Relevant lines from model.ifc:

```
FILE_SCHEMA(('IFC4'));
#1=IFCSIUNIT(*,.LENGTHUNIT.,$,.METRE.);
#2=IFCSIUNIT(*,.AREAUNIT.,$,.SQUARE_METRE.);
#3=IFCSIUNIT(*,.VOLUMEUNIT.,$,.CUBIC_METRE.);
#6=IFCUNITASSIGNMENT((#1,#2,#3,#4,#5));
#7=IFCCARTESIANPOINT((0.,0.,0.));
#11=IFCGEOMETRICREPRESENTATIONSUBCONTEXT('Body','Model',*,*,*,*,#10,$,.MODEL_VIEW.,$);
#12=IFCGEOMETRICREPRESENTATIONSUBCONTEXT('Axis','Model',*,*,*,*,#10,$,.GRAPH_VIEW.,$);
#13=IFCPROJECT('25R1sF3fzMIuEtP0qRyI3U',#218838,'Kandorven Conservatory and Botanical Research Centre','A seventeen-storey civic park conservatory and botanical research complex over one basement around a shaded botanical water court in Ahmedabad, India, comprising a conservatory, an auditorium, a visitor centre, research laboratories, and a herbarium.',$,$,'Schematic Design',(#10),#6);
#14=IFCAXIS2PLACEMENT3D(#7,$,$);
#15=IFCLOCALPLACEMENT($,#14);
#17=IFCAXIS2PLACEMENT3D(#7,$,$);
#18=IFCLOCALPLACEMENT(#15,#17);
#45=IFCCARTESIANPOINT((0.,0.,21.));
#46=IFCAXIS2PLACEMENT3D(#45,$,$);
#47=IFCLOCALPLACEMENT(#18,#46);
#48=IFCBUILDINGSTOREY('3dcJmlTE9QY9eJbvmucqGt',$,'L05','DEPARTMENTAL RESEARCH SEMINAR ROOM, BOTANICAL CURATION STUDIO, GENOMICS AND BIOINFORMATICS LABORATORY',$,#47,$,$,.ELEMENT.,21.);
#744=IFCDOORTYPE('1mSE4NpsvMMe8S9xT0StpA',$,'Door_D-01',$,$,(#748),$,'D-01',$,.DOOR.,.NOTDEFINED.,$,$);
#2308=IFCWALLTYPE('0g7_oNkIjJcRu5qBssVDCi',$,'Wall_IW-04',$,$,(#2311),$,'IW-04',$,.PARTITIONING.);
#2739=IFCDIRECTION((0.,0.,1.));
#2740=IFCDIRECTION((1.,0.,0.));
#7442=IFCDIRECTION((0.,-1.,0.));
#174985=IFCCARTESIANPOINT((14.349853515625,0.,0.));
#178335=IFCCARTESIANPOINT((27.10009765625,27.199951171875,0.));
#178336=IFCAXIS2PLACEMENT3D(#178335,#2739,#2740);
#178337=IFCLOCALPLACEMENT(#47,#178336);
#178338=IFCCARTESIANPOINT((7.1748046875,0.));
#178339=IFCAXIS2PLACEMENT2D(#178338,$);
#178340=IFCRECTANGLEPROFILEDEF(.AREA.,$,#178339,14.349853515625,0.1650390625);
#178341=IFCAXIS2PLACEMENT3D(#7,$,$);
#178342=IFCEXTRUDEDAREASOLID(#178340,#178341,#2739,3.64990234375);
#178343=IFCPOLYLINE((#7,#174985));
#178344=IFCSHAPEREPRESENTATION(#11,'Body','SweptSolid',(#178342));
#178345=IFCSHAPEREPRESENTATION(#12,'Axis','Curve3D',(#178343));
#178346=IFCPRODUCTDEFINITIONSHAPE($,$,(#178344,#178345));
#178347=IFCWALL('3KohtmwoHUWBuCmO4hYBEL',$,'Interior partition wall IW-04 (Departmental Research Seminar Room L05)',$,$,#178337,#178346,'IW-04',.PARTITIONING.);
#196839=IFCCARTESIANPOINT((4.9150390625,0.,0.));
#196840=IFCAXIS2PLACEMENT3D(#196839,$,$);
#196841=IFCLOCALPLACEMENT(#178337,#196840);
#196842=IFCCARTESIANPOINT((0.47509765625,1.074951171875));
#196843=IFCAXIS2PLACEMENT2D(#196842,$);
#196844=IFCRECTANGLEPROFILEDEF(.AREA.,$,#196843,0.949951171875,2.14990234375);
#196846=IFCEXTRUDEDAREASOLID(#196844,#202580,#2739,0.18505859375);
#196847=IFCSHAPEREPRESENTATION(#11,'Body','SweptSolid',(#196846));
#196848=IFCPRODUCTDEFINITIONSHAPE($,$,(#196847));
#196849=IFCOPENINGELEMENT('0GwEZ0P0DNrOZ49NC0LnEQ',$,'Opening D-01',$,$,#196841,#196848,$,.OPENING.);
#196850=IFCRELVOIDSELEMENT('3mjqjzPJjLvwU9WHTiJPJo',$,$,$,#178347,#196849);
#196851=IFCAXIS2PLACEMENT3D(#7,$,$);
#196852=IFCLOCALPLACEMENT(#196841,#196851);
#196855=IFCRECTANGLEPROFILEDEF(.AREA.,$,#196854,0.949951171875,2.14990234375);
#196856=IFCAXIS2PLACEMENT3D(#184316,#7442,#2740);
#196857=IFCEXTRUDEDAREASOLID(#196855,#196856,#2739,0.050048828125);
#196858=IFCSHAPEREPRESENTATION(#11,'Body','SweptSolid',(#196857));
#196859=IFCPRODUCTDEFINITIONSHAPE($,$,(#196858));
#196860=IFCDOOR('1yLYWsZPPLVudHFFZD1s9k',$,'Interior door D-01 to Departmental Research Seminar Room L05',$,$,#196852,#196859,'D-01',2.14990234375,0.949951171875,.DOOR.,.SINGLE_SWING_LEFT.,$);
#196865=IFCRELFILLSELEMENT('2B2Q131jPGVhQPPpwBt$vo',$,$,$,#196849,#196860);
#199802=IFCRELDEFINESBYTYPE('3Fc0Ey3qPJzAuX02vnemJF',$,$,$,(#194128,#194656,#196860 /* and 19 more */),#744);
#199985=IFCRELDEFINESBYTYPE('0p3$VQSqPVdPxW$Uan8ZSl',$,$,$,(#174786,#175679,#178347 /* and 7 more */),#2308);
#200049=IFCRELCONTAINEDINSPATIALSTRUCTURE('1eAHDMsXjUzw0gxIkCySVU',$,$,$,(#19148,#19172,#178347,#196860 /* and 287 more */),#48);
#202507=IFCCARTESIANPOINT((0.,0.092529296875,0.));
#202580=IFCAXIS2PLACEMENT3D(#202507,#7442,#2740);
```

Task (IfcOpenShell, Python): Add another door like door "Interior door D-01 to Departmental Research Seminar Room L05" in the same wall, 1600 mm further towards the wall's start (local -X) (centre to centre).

```python
import ifcopenshell
import ifcopenshell.api.feature
import ifcopenshell.api.geometry
import ifcopenshell.api.root
import ifcopenshell.geom
import ifcopenshell.util.element
import ifcopenshell.util.placement
import ifcopenshell.util.shape
import ifcopenshell.util.unit

model = ifcopenshell.open("model.ifc")
unit_scale = ifcopenshell.util.unit.calculate_unit_scale(model)
settings = ifcopenshell.geom.settings()


def volume(element):
    """Net volume in cubic metres, openings subtracted."""
    shape = ifcopenshell.geom.create_shape(settings, element)
    return ifcopenshell.util.shape.get_volume(shape.geometry)


door = model.by_guid("1yLYWsZPPLVudHFFZD1s9k")
opening = door.FillsVoids[0].RelatingOpeningElement
wall = opening.VoidsElements[0].RelatingBuildingElement
before = volume(wall)
shift = ifcopenshell.util.placement.get_local_placement(wall.ObjectPlacement)[:3, 0] * -1.6 / unit_scale

# copy_class copies the void relationship, type, container and properties, but no geometry.
new_opening = ifcopenshell.api.root.copy_class(model, product=opening)
new_opening.Representation = ifcopenshell.util.element.copy_deep(
    model, opening.Representation, exclude=["IfcGeometricRepresentationContext", "IfcRepresentationMap"]
)
new_door = ifcopenshell.api.root.copy_class(model, product=door)
new_door.Representation = ifcopenshell.util.element.copy_deep(
    model, door.Representation, exclude=["IfcGeometricRepresentationContext", "IfcRepresentationMap"]
)
new_door.Tag = None
ifcopenshell.api.feature.add_filling(model, opening=new_opening, element=new_door)

for old, new in ((opening, new_opening), (door, new_door)):
    matrix = ifcopenshell.util.placement.get_local_placement(old.ObjectPlacement)
    matrix[:3, 3] += shift
    ifcopenshell.api.geometry.edit_object_placement(model, product=new, matrix=matrix, is_si=False)

after = volume(wall)

print(f"wall volume {before:.3f} -> {after:.3f} m3")

model.write("model-out.ifc")
```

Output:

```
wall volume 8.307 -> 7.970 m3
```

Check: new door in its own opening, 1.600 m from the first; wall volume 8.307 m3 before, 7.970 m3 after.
